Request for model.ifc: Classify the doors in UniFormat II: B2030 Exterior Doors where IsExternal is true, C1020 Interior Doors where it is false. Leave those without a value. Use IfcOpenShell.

First a look at what the model holds.

```python
import ifcopenshell
import ifcopenshell.util.element

model = ifcopenshell.open("model.ifc")
print(model.schema)
print("classifications:", [c.Name for c in model.by_type("IfcClassification")])
values = [ifcopenshell.util.element.get_pset(e, "Pset_DoorCommon", "IsExternal") for e in model.by_type("IfcDoor")]
for value in (True, False, None):
    print("IsExternal", value, values.count(value))
```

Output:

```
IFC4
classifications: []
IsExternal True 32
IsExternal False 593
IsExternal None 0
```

```python
import ifcopenshell
import ifcopenshell.api.classification
import ifcopenshell.util.element

model = ifcopenshell.open("model.ifc")

system = ifcopenshell.api.classification.add_classification(model, classification="UniFormat II")

doors = model.by_type("IfcDoor")
external = {e: ifcopenshell.util.element.get_pset(e, "Pset_DoorCommon", "IsExternal") for e in doors}
for flag, code, name in ((True, "B2030", "Exterior Doors"), (False, "C1020", "Interior Doors")):
    products = [e for e in doors if external[e] is flag]
    ifcopenshell.api.classification.add_reference(
        model, products=products, classification=system, identification=code, name=name
    )
    print(code, len(products))

model.write("model_rev.ifc")
```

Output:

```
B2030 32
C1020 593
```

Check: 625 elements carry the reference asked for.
